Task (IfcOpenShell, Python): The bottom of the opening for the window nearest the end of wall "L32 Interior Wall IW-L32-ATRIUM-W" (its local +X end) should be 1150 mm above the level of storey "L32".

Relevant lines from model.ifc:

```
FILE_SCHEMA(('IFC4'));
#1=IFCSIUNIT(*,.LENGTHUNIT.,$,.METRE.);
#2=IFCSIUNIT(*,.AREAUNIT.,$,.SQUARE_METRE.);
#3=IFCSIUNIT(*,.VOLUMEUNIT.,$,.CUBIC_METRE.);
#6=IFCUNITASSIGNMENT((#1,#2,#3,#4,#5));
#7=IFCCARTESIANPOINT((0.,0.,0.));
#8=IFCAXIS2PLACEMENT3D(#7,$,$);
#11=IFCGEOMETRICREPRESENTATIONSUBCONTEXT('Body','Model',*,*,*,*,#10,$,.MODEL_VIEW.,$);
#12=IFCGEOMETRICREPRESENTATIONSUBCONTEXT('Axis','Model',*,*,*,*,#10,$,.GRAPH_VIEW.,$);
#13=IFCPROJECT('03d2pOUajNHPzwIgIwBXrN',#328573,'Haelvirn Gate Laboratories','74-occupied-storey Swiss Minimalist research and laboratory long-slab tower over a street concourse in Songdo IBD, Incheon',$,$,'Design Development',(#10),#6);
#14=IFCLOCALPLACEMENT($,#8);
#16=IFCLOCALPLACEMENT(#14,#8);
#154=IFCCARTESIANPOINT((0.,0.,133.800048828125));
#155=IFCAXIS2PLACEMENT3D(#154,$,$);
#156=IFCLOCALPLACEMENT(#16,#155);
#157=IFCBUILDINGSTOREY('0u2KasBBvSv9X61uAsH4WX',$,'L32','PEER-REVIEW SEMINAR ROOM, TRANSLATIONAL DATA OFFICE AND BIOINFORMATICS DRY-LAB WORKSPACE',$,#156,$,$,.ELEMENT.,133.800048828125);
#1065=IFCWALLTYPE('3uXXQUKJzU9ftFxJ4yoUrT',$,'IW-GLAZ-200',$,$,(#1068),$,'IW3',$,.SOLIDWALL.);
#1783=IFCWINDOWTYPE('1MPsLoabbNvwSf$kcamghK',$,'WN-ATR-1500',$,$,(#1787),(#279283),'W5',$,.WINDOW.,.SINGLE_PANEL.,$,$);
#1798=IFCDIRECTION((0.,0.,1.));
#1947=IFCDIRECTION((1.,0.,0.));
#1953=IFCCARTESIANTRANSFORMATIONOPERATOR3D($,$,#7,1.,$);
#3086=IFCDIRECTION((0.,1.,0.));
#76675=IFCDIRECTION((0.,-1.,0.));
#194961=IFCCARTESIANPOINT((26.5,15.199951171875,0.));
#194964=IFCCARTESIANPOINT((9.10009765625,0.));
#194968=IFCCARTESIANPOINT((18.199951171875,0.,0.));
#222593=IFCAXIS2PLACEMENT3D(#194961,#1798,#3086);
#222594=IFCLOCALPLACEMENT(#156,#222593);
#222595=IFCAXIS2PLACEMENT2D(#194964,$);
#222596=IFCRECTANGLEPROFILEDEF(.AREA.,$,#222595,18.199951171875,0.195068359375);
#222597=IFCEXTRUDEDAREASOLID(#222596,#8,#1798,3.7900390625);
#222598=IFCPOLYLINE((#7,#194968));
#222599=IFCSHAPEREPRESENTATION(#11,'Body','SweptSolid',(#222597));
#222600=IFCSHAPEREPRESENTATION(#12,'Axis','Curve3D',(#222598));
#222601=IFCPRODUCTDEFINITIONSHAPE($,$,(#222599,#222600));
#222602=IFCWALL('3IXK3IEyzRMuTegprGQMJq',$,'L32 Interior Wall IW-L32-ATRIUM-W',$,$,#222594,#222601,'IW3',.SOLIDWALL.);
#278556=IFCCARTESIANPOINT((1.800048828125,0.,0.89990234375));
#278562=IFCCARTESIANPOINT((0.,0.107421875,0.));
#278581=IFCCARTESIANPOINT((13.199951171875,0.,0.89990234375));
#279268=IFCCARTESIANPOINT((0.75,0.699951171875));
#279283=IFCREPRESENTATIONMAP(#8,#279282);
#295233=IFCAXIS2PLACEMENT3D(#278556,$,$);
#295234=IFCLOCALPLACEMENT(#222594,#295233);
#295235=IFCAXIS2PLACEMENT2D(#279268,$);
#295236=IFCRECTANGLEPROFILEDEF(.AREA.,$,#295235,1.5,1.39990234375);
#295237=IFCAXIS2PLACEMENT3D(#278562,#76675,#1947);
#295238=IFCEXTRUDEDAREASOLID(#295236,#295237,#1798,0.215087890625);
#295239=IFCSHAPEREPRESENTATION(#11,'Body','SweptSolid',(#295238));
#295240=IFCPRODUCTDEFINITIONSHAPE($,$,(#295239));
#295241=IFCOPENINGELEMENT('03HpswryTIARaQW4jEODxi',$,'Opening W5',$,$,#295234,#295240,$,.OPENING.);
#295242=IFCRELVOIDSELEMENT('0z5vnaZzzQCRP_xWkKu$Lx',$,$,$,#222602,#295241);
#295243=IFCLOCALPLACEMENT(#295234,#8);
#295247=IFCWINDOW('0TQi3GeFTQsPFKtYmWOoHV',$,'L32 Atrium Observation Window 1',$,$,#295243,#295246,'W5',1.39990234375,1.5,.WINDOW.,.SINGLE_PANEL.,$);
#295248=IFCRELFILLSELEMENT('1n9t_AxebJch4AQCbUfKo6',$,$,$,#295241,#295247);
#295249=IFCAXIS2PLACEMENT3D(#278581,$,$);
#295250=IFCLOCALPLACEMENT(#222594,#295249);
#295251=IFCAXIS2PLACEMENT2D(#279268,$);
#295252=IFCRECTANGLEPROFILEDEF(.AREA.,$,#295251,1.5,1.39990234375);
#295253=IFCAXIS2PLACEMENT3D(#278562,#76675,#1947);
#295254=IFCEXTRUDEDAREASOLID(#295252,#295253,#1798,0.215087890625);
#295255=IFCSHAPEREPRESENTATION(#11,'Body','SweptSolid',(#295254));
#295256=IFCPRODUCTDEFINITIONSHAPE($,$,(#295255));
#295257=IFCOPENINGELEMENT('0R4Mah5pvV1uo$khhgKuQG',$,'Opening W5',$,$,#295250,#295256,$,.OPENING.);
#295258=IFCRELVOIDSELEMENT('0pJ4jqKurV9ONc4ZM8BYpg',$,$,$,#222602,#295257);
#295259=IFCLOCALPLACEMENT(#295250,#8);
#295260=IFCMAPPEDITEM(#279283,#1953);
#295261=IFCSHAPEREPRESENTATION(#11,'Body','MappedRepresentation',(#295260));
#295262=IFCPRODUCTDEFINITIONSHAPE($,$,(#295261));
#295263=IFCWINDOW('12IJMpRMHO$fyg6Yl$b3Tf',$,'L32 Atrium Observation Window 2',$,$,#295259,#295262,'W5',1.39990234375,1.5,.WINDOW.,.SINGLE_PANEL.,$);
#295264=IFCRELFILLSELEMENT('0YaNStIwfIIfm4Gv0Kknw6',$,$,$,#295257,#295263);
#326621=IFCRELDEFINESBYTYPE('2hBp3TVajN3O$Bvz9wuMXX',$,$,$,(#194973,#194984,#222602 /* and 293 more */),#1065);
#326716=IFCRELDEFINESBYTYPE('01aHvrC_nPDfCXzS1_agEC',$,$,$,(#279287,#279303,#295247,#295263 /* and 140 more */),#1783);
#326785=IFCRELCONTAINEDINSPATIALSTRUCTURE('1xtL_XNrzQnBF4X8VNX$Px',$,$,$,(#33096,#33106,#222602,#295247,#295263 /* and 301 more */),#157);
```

```python
import numpy as np
import ifcopenshell
import ifcopenshell.api.geometry
import ifcopenshell.geom
import ifcopenshell.util.element
import ifcopenshell.util.placement
import ifcopenshell.util.shape
import ifcopenshell.util.unit

model = ifcopenshell.open("model.ifc")
unit_scale = ifcopenshell.util.unit.calculate_unit_scale(model)

window = model.by_guid("12IJMpRMHO$fyg6Yl$b3Tf")
opening = window.FillsVoids[0].RelatingOpeningElement
storey = ifcopenshell.util.element.get_container(window, ifc_class="IfcBuildingStorey")
level = ifcopenshell.util.placement.get_local_placement(storey.ObjectPlacement)[2, 3]

# The opening's origin need not be at the sill, so measure its lowest point.
shape = ifcopenshell.geom.create_shape(ifcopenshell.geom.settings(), opening)
bottom = ifcopenshell.util.shape.get_shape_bottom_elevation(shape, shape.geometry) / unit_scale
dz = level + 1.15 / unit_scale - bottom

shift = np.array([0.0, 0.0, dz])
# The window is placed relative to its opening, so it follows when the opening moves.
matrix = ifcopenshell.util.placement.get_local_placement(opening.ObjectPlacement)
matrix[:3, 3] += shift
ifcopenshell.api.geometry.edit_object_placement(
    model, product=opening, matrix=matrix, is_si=False, should_transform_children=True
)

print(f"moved by {dz * unit_scale:+.3f} m")

model.write("model_rev.ifc")
```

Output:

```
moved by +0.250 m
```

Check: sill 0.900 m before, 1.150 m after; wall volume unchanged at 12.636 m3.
